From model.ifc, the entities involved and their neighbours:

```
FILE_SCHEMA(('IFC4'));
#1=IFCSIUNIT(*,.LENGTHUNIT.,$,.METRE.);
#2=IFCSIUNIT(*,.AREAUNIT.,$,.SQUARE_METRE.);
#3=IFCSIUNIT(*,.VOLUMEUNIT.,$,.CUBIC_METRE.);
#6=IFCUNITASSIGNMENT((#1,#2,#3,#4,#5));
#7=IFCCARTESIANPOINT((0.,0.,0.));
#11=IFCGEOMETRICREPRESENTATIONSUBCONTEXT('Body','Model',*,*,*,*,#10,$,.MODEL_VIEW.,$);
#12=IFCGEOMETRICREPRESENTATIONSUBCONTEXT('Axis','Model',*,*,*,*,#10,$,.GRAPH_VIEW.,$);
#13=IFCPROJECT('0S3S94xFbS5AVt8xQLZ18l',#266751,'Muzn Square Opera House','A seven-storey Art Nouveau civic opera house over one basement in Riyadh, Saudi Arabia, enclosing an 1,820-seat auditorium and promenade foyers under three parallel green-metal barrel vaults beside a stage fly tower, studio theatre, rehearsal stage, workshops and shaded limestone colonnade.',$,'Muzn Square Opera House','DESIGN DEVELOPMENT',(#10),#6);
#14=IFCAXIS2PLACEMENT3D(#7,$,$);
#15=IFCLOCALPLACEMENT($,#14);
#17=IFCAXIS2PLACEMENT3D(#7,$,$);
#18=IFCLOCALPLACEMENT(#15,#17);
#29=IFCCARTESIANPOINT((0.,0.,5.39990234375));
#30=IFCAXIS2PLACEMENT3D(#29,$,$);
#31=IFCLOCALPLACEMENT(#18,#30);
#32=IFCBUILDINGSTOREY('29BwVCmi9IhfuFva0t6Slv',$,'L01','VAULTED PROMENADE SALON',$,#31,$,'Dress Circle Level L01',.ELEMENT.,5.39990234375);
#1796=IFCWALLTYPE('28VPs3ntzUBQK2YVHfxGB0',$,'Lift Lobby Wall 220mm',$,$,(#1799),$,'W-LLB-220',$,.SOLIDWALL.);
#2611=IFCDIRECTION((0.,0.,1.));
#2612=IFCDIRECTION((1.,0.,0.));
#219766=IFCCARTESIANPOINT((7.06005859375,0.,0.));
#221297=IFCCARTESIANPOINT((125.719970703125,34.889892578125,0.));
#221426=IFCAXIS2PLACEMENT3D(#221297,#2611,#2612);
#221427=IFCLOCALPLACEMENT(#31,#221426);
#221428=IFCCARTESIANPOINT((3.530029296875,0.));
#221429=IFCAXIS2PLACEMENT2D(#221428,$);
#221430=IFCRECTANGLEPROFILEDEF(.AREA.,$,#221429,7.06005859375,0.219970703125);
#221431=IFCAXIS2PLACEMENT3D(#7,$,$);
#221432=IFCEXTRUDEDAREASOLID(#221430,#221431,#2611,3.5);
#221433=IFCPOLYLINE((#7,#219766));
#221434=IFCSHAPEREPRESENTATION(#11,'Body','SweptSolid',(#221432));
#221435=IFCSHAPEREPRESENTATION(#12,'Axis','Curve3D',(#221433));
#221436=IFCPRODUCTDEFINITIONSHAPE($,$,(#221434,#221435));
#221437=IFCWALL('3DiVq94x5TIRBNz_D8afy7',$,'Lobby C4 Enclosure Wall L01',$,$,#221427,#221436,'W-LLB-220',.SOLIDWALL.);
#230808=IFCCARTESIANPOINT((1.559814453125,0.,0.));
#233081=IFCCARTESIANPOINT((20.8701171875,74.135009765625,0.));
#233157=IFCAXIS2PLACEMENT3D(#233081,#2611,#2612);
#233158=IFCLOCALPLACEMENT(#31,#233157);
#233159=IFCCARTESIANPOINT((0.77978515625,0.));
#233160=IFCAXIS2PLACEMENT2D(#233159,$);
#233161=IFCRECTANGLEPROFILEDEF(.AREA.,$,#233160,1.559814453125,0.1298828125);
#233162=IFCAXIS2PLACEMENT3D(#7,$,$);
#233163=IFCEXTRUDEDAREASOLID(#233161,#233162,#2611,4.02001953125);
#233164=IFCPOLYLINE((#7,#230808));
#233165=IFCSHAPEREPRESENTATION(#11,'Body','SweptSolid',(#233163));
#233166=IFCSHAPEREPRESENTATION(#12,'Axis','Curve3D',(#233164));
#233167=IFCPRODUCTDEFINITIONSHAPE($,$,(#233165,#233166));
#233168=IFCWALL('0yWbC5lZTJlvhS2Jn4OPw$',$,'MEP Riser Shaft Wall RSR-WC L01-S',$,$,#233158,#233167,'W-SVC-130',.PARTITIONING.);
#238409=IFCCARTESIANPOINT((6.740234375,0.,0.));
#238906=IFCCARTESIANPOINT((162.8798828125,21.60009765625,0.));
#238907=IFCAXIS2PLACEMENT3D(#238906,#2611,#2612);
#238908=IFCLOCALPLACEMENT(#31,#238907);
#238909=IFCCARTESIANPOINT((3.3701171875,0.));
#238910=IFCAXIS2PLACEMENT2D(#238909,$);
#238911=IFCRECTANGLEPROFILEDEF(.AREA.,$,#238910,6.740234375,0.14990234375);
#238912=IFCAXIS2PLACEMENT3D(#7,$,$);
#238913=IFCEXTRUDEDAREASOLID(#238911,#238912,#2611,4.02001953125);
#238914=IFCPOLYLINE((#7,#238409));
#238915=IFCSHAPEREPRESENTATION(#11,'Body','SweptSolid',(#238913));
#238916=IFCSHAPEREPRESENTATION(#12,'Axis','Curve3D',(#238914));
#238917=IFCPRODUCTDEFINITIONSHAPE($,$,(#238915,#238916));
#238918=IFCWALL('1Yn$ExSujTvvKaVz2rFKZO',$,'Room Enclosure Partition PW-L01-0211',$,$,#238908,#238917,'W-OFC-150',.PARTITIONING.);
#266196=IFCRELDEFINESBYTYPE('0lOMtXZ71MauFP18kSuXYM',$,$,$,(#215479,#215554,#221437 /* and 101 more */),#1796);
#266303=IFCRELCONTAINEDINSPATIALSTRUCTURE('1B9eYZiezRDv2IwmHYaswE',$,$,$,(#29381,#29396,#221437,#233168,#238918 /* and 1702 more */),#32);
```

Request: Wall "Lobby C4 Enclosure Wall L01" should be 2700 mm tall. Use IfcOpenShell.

```python
import ifcopenshell
import ifcopenshell.geom
import ifcopenshell.util.representation
import ifcopenshell.util.shape
import ifcopenshell.util.unit

model = ifcopenshell.open("model.ifc")
unit_scale = ifcopenshell.util.unit.calculate_unit_scale(model)
settings = ifcopenshell.geom.settings()


def volume(element):
    """Net volume in cubic metres, openings subtracted."""
    shape = ifcopenshell.geom.create_shape(settings, element)
    return ifcopenshell.util.shape.get_volume(shape.geometry)


wall = model.by_id(221437)
before = volume(wall)

body = ifcopenshell.util.representation.get_representation(wall, "Model", "Body")
solid = body.Items[0]
old_height = solid.Depth
solid.Depth = 2.7 / unit_scale
after = volume(wall)

print(f"height {old_height:g} -> {solid.Depth:g}, volume {before:.3f} -> {after:.3f} m3")

model.write("model_rev.ifc")
```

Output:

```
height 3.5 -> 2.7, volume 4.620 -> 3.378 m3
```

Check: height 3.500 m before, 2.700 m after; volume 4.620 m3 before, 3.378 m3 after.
